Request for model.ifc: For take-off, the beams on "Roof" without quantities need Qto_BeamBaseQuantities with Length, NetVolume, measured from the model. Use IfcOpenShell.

First a look at what the model holds.

```python
import ifcopenshell
import ifcopenshell.util.element
import ifcopenshell.util.unit

model = ifcopenshell.open("model.ifc")
print(model.schema)
for unit_type in ("LENGTHUNIT", "AREAUNIT", "VOLUMEUNIT"):
    print(unit_type, ifcopenshell.util.unit.calculate_unit_scale(model, unit_type))
storey = next(s for s in model.by_type("IfcBuildingStorey") if s.Name == "Roof")
beams = [e for e in ifcopenshell.util.element.get_decomposition(storey) if e.is_a("IfcBeam")]
for e in sorted(beams, key=lambda e: e.id()):
    print(e.id(), e.is_a(), e.Name, list(ifcopenshell.util.element.get_psets(e, qtos_only=True)), sep=" | ")
```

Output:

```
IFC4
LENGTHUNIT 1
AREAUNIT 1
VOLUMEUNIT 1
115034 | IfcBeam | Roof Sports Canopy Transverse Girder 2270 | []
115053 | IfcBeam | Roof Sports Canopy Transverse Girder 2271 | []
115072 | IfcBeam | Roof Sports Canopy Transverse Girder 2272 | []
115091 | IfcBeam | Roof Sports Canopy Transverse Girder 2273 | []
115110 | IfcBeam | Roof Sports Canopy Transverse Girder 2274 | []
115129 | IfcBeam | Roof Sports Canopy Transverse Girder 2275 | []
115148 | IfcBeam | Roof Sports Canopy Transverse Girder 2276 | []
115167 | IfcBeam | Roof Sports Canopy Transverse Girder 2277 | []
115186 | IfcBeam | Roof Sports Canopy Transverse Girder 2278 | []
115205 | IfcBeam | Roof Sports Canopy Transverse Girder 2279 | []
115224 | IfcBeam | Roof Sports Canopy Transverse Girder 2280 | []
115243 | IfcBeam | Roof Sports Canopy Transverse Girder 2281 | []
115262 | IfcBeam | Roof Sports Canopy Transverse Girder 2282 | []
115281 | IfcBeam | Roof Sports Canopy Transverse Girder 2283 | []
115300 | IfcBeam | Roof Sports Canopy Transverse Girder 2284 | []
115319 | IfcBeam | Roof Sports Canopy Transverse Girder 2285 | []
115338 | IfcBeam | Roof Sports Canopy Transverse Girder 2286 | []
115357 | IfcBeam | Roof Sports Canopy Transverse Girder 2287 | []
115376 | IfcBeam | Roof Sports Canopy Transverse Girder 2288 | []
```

```python
import ifcopenshell
import ifcopenshell.api.pset
import ifcopenshell.geom
import ifcopenshell.util.element
import ifcopenshell.util.shape
import ifcopenshell.util.unit

model = ifcopenshell.open("model.ifc")
unit_scale = ifcopenshell.util.unit.calculate_unit_scale(model)
volume_scale = ifcopenshell.util.unit.calculate_unit_scale(model, "VOLUMEUNIT")
settings = ifcopenshell.geom.settings()

storey = next(s for s in model.by_type("IfcBuildingStorey") if s.Name == "Roof")
beams = [e for e in ifcopenshell.util.element.get_decomposition(storey) if e.is_a("IfcBeam")]

for e in sorted(beams, key=lambda e: e.id()):
    if ifcopenshell.util.element.get_psets(e, qtos_only=True, should_inherit=False):
        continue
    # Geometry comes back in metres, in the element's own axes.
    shape = ifcopenshell.geom.create_shape(settings, e)
    values = {
        "Length": ifcopenshell.util.shape.get_max_xyz(shape.geometry) / unit_scale,
        "NetVolume": ifcopenshell.util.shape.get_volume(shape.geometry) / volume_scale,
    }
    qto = ifcopenshell.api.pset.add_qto(model, product=e, name="Qto_BeamBaseQuantities")
    ifcopenshell.api.pset.edit_qto(model, qto=qto, properties=values)
    print(e.id(), {k: round(v, 3) for k, v in values.items()})

model.write("model_rev.ifc")
```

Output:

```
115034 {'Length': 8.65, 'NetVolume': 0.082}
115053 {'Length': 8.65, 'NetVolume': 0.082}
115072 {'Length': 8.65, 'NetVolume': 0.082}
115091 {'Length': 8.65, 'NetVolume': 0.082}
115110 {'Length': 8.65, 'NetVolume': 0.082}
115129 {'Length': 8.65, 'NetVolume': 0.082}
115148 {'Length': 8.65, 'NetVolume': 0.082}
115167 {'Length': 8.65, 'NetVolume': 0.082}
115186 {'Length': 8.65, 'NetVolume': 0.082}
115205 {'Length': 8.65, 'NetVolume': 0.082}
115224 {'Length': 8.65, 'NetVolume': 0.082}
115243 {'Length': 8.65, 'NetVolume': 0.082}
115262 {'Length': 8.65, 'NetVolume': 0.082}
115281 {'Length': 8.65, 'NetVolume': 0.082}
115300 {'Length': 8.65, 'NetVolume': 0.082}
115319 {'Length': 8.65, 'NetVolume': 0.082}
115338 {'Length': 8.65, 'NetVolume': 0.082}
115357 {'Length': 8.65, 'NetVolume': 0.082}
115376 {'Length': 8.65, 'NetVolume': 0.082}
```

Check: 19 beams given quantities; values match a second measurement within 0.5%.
